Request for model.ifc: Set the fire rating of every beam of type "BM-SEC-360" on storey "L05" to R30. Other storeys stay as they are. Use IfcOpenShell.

First a look at what the model holds.

```python
import ifcopenshell
import ifcopenshell.util.element

model = ifcopenshell.open("model.ifc")
print(model.schema)
storey = next(s for s in model.by_type("IfcBuildingStorey") if s.Name == "L05")
beams = [e for e in ifcopenshell.util.element.get_decomposition(storey) if e.is_a("IfcBeam")]
seen = {}
for e in beams:
    element_type = ifcopenshell.util.element.get_type(e)
    key = (element_type.Name if element_type != e and element_type else None, ifcopenshell.util.element.get_pset(e, "Pset_BeamCommon", "FireRating"))
    seen[key] = seen.get(key, 0) + 1
for (name, value), count in sorted(seen.items(), key=str):
    print(count, "x", name, "|", value)
```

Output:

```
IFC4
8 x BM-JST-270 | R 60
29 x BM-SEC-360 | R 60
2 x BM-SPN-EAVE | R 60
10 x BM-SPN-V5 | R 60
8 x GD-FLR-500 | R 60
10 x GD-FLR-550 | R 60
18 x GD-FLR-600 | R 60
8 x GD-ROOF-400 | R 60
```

```python
import ifcopenshell
import ifcopenshell.api.pset
import ifcopenshell.util.element

model = ifcopenshell.open("model.ifc")

storey = next(s for s in model.by_type("IfcBuildingStorey") if s.Name == "L05")
beams = [e for e in ifcopenshell.util.element.get_decomposition(storey) if e.is_a("IfcBeam")]

count = 0
for e in beams:
    element_type = ifcopenshell.util.element.get_type(e)
    if element_type in (None, e) or element_type.Name != "BM-SEC-360":
        continue
    # add_pset returns the element's existing set when there is one.
    pset = ifcopenshell.api.pset.add_pset(model, product=e, name="Pset_BeamCommon")
    ifcopenshell.api.pset.edit_pset(model, pset=pset, properties={"FireRating": "R30"})
    count += 1

print(count, "beams updated")

model.write("model_v2.ifc")
```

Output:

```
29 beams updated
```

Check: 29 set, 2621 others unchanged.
